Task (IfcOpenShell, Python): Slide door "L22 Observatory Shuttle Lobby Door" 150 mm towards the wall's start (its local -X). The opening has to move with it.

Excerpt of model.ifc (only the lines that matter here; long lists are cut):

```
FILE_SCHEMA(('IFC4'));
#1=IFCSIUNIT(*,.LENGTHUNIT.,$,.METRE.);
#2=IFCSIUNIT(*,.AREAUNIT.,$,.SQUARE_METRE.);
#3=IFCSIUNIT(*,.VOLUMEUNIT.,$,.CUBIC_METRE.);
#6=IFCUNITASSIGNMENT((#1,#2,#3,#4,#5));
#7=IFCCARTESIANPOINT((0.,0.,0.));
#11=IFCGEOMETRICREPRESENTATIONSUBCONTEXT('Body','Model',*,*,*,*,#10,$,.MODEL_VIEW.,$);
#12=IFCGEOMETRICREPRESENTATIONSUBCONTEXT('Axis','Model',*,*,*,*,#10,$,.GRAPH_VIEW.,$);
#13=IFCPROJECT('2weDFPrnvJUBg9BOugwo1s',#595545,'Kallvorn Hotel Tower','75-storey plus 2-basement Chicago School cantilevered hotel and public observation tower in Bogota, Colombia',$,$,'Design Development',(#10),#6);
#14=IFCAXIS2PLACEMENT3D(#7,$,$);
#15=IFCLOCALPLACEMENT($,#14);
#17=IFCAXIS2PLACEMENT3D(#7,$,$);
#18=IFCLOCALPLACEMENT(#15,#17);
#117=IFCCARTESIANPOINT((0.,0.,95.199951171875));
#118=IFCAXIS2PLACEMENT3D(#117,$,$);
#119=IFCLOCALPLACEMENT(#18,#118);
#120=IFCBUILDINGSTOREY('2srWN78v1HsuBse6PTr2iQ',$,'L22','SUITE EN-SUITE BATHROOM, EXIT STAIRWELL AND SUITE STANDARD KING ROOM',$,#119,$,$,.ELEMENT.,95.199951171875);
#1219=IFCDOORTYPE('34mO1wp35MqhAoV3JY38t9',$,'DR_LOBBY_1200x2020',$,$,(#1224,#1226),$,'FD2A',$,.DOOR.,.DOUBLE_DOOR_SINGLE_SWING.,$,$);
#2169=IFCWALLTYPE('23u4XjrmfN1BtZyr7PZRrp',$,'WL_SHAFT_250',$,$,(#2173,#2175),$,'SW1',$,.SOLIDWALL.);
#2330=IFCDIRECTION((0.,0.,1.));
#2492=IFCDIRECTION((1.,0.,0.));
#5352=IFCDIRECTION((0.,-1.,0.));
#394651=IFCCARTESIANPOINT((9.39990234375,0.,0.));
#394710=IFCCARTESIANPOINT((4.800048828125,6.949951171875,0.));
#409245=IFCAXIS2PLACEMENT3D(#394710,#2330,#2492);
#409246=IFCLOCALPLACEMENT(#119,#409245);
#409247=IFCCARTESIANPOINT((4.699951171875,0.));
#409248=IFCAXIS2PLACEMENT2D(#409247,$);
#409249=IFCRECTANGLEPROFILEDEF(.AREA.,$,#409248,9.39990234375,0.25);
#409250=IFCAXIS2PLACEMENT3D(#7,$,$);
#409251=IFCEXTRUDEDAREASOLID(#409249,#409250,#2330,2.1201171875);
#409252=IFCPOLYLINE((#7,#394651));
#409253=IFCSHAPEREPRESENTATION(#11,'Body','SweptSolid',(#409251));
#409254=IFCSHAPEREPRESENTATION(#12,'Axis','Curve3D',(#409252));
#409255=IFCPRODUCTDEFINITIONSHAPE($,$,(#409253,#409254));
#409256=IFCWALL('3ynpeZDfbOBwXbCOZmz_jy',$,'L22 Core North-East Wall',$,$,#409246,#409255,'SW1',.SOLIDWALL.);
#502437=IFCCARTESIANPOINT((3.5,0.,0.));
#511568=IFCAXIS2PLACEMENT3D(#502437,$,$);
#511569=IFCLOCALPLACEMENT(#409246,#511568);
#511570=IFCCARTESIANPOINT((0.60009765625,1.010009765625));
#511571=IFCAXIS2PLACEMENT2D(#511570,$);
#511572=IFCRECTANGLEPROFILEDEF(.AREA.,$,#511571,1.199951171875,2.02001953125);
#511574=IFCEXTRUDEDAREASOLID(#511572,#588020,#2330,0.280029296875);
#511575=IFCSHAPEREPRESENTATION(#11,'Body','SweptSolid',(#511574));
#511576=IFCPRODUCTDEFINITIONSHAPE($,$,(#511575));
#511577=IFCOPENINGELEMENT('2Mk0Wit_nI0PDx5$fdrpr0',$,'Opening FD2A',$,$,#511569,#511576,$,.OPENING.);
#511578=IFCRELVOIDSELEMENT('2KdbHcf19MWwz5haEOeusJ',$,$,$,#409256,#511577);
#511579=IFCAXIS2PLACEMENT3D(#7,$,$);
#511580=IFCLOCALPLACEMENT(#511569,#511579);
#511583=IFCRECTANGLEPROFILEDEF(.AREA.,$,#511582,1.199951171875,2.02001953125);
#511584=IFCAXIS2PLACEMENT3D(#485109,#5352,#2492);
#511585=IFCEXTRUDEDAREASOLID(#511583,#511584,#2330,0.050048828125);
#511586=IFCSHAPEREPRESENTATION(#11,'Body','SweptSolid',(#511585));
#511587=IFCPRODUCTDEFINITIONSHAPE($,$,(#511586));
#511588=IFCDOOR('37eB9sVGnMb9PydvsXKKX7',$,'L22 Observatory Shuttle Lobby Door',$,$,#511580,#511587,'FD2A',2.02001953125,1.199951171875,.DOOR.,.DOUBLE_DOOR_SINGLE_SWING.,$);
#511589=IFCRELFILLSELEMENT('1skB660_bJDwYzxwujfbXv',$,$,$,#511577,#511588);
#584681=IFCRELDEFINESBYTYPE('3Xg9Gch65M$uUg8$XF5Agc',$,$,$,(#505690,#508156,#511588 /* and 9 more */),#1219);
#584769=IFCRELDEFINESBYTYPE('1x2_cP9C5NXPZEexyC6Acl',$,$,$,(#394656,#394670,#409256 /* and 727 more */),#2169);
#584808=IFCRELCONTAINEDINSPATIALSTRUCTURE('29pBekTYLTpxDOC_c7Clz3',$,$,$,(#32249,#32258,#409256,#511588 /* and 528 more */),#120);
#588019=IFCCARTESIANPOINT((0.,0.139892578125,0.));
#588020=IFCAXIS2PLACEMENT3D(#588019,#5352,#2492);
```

```python
import ifcopenshell
import ifcopenshell.api.geometry
import ifcopenshell.util.placement

model = ifcopenshell.open("model.ifc")

door = model.by_guid("37eB9sVGnMb9PydvsXKKX7")
opening = door.FillsVoids[0].RelatingOpeningElement
wall = opening.VoidsElements[0].RelatingBuildingElement

wall_matrix = ifcopenshell.util.placement.get_local_placement(wall.ObjectPlacement)
shift = wall_matrix[:3, 0] * -0.15
before = ifcopenshell.util.placement.get_local_placement(door.ObjectPlacement)[:3, 3].copy()

# The door is placed relative to its opening, so it follows when the opening moves.
matrix = ifcopenshell.util.placement.get_local_placement(opening.ObjectPlacement)
matrix[:3, 3] += shift
ifcopenshell.api.geometry.edit_object_placement(
    model, product=opening, matrix=matrix, is_si=False, should_transform_children=True
)

after = ifcopenshell.util.placement.get_local_placement(door.ObjectPlacement)[:3, 3]
print("door moved by", (after - before).round(3) + 0.0)

model.write("model_updated.ifc")
```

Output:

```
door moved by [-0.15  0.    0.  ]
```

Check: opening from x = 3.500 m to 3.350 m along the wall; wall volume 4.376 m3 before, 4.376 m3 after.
